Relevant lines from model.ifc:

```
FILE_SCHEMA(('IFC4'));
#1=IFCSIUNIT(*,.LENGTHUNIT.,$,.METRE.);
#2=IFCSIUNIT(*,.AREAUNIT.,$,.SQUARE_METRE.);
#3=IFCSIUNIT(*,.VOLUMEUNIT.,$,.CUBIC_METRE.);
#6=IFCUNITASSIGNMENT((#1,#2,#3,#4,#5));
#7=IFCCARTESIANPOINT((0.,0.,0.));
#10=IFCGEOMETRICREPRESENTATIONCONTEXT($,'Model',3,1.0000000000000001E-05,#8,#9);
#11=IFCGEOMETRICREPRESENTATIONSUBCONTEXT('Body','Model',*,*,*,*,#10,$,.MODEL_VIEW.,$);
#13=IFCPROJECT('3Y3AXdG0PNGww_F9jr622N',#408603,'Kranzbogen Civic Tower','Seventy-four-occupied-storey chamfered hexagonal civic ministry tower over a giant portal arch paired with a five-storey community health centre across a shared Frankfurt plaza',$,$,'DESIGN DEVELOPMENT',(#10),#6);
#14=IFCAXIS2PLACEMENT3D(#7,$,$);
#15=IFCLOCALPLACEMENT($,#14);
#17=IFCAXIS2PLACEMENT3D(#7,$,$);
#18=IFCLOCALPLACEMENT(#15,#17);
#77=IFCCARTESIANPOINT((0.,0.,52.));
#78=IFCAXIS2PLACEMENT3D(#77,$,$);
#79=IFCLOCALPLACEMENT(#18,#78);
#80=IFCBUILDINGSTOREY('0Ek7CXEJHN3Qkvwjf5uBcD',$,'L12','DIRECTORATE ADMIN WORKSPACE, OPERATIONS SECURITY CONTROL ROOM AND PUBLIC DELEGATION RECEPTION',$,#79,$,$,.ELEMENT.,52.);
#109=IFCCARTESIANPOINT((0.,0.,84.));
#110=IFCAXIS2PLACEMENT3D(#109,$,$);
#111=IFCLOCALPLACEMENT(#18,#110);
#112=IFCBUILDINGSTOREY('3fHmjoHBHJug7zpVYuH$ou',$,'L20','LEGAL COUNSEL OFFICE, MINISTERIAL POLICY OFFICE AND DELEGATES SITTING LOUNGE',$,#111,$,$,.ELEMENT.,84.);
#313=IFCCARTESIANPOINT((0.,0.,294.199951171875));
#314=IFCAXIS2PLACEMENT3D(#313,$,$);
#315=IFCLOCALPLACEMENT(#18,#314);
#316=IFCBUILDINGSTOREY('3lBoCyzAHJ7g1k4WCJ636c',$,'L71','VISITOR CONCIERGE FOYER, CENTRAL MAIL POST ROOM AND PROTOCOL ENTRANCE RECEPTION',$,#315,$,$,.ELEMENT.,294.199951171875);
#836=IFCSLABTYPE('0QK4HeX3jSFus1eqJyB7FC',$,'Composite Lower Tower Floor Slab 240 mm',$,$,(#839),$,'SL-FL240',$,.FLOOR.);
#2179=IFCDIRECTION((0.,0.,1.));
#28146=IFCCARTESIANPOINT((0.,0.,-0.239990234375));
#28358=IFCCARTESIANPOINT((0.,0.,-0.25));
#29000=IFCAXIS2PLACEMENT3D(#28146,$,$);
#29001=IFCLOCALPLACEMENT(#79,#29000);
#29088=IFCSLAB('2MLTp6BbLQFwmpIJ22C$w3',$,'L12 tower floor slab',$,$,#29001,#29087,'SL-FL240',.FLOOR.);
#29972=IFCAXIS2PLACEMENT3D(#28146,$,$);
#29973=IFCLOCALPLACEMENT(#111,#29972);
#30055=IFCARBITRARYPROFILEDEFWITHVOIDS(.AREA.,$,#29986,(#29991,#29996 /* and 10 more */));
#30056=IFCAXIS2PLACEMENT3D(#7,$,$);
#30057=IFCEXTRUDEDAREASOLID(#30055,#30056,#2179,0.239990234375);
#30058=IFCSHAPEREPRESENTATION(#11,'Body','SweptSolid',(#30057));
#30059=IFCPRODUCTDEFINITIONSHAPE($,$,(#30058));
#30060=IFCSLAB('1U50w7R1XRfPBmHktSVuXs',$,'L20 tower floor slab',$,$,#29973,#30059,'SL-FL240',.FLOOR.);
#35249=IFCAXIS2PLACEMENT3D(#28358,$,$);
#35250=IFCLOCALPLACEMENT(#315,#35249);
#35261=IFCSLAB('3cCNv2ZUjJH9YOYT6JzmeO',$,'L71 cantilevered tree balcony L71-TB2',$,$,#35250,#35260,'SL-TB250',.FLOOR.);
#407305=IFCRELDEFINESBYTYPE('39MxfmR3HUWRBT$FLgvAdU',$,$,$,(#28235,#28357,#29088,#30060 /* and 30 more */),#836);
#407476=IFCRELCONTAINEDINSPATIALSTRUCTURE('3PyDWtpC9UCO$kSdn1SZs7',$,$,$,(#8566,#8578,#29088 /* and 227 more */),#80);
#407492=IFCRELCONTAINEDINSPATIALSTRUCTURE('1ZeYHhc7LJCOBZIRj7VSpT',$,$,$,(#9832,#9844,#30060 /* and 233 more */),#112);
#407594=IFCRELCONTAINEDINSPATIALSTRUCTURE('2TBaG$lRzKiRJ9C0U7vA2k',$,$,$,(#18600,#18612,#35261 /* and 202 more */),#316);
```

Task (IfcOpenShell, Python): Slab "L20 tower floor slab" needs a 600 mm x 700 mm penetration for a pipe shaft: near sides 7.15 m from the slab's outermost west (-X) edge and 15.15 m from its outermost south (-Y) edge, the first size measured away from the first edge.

```python
import numpy as np
import ifcopenshell
import ifcopenshell.api.feature
import ifcopenshell.api.geometry
import ifcopenshell.api.root
import ifcopenshell.geom
import ifcopenshell.util.placement
import ifcopenshell.util.representation
import ifcopenshell.util.shape
import ifcopenshell.util.unit

model = ifcopenshell.open("model.ifc")
unit_scale = ifcopenshell.util.unit.calculate_unit_scale(model)
settings = ifcopenshell.geom.settings()


def volume(element):
    """Net volume in cubic metres, openings subtracted."""
    shape = ifcopenshell.geom.create_shape(settings, element)
    return ifcopenshell.util.shape.get_volume(shape.geometry)


slab = model.by_id(30060)
before = volume(slab)

# Extent in the slab's own axes, in metres. The edges named are its -X and -Y sides.
slab_shape = ifcopenshell.geom.create_shape(settings, slab)
vertices = ifcopenshell.util.shape.get_vertices(slab_shape.geometry)
x_min, y_min, bottom = vertices.min(axis=0)
top = vertices[:, 2].max()

opening = ifcopenshell.api.root.create_entity(model, ifc_class="IfcOpeningElement", name="Pipe shaft opening", predefined_type="OPENING")
context = ifcopenshell.util.representation.get_context(model, "Model", "Body", "MODEL_VIEW")
width, depth = 0.6, 0.7
outline = [(0.0, 0.0), (width, 0.0), (width, depth), (0.0, depth), (0.0, 0.0)]
# Overshoot both faces by 50 mm so the cut is clean.
shape = ifcopenshell.api.geometry.add_slab_representation(
    model, context=context, depth=top - bottom + 0.1, polyline=outline
)
ifcopenshell.api.geometry.assign_representation(model, product=opening, representation=shape)

matrix = ifcopenshell.util.placement.get_local_placement(slab.ObjectPlacement)
matrix[:, 3] = matrix @ np.append(np.array([x_min + 7.15, y_min + 15.15, bottom - 0.05]) / unit_scale, 1.0)
ifcopenshell.api.geometry.edit_object_placement(model, product=opening, matrix=matrix, is_si=False)
ifcopenshell.api.feature.add_feature(model, feature=opening, element=slab)

after = volume(slab)

print(f"slab volume {before:.3f} -> {after:.3f} m3")

model.write("model_updated.ifc")
```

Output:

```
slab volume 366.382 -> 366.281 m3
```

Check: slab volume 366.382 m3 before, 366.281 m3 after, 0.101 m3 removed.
